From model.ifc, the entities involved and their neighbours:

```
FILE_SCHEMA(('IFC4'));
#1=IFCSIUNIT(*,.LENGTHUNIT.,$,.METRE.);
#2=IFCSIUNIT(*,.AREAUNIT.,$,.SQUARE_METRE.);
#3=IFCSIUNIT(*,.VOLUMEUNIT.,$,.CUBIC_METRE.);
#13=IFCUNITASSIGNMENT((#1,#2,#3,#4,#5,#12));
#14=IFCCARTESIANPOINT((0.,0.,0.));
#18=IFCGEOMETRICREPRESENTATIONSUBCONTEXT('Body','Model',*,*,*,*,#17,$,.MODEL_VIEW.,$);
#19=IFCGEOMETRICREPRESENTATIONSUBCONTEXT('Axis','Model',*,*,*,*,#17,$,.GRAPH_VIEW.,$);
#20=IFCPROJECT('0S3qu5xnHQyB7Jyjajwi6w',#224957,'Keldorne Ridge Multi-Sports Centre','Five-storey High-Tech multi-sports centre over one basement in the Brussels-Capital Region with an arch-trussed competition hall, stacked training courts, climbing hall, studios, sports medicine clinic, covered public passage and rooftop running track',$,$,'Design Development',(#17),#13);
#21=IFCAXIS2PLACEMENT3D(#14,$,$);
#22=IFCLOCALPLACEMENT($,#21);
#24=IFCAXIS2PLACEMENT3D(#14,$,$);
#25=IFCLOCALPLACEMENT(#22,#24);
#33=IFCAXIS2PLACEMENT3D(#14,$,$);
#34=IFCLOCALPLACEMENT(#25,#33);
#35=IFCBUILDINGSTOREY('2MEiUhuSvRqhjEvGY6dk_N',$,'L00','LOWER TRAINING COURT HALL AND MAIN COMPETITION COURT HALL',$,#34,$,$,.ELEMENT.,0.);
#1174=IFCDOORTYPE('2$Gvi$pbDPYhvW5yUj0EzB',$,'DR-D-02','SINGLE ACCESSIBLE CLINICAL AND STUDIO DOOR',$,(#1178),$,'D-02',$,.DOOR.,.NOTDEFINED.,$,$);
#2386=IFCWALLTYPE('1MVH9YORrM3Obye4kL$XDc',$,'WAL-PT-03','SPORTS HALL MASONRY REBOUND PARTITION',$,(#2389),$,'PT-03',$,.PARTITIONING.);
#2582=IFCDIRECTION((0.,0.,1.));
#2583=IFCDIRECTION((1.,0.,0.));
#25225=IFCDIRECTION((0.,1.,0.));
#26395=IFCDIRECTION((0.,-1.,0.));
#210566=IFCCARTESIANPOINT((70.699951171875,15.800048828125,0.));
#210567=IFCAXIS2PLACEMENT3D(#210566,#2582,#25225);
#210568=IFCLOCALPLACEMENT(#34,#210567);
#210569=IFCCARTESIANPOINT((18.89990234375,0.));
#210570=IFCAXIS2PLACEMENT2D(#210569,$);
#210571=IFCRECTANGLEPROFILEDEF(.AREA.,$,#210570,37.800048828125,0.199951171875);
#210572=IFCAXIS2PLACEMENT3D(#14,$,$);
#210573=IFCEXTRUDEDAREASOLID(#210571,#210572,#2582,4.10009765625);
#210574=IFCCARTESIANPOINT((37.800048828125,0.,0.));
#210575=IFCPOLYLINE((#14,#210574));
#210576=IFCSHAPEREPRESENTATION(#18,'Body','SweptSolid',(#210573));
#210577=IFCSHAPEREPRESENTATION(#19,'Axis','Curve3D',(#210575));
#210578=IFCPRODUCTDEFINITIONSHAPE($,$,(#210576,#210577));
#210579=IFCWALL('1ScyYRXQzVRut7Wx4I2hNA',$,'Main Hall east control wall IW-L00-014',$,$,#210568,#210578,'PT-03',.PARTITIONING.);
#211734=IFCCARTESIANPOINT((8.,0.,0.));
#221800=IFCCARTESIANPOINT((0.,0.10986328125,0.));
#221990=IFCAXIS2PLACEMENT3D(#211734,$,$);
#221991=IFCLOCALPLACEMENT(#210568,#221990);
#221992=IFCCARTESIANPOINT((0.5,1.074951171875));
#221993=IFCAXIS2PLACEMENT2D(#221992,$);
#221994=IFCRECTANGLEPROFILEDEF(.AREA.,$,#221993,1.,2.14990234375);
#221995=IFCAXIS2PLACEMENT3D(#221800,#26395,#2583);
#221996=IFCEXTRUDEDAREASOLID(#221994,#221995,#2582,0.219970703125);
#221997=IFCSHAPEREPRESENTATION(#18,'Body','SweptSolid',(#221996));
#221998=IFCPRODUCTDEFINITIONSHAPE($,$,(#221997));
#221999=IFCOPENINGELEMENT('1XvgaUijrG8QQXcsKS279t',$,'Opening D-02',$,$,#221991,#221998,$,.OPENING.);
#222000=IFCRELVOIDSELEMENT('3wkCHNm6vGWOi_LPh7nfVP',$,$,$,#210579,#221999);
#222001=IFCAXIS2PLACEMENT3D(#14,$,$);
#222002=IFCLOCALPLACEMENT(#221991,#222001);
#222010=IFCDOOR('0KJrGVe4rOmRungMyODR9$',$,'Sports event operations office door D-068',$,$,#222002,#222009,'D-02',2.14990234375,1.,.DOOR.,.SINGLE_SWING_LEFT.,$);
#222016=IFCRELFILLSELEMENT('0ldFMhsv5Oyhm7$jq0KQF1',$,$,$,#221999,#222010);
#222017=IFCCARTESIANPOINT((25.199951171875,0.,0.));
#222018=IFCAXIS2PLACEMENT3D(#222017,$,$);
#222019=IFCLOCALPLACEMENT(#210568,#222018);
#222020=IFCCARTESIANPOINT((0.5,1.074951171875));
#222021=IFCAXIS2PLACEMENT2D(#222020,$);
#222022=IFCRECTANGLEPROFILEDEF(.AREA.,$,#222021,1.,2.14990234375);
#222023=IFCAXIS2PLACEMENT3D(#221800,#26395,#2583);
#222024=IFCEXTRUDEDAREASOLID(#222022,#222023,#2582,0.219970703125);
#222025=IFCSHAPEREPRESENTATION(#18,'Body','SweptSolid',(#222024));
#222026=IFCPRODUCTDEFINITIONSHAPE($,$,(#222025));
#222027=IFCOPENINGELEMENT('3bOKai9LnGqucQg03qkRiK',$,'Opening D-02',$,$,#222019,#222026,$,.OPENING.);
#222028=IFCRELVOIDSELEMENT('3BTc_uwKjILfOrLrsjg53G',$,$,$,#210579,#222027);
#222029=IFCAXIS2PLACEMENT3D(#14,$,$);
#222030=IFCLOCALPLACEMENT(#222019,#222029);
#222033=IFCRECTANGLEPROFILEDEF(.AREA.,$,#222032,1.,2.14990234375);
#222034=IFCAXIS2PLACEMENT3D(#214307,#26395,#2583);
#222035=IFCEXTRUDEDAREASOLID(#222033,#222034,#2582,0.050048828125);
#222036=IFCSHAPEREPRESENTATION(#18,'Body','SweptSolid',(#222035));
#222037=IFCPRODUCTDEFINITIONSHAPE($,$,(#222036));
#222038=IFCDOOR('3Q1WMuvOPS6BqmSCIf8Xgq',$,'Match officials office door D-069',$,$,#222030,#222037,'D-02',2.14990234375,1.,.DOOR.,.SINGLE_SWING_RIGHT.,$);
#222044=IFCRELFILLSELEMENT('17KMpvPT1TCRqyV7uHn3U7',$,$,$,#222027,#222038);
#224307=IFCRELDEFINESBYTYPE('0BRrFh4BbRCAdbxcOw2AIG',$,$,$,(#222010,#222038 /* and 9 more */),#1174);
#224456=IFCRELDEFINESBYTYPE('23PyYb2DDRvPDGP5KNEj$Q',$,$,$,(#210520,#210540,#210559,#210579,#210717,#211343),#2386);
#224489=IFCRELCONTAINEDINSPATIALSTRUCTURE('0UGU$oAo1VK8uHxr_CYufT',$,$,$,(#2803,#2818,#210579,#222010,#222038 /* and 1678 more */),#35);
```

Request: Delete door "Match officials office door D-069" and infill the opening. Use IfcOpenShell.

```python
import ifcopenshell
import ifcopenshell.api.feature
import ifcopenshell.api.root
import ifcopenshell.geom
import ifcopenshell.util.shape

model = ifcopenshell.open("model.ifc")
settings = ifcopenshell.geom.settings()


def volume(element):
    """Net volume in cubic metres, openings subtracted."""
    shape = ifcopenshell.geom.create_shape(settings, element)
    return ifcopenshell.util.shape.get_volume(shape.geometry)


door = model.by_guid("3Q1WMuvOPS6BqmSCIf8Xgq")
opening = door.FillsVoids[0].RelatingOpeningElement
wall = opening.VoidsElements[0].RelatingBuildingElement
before = volume(wall)

ifcopenshell.api.root.remove_product(model, product=door)
ifcopenshell.api.feature.remove_feature(model, feature=opening)

after = volume(wall)

print(f"wall volume {before:.3f} -> {after:.3f} m3")

model.write("model_v2.ifc")
```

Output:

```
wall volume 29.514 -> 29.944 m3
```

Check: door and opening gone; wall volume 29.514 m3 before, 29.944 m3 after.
